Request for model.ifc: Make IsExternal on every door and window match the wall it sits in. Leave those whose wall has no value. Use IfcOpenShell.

First a look at what the model holds.

```python
import ifcopenshell
import ifcopenshell.util.element

model = ifcopenshell.open("model.ifc")
print(model.schema)
seen = {}
for e in model.by_type("IfcDoor") + model.by_type("IfcWindow"):
    if not e.FillsVoids:
        continue
    host = e.FillsVoids[0].RelatingOpeningElement.VoidsElements[0].RelatingBuildingElement
    own = ifcopenshell.util.element.get_pset(e, f"Pset_{e.is_a()[3:].removesuffix('StandardCase')}Common", "IsExternal")
    wall = ifcopenshell.util.element.get_pset(host, "Pset_WallCommon", "IsExternal")
    seen[e.is_a(), own, wall] = seen.get((e.is_a(), own, wall), 0) + 1
for (cls, own, wall), count in sorted(seen.items(), key=str):
    print(count, cls, "IsExternal:", own, "| host wall:", wall)
```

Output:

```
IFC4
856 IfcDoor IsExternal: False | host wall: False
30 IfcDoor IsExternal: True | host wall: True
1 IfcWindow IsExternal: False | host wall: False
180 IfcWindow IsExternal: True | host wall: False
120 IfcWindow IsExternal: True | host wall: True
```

```python
import ifcopenshell
import ifcopenshell.api.pset
import ifcopenshell.util.element

model = ifcopenshell.open("model.ifc")

count = 0
for ifc_class, pset_name in (("IfcDoor", "Pset_DoorCommon"), ("IfcWindow", "Pset_WindowCommon")):
    for e in model.by_type(ifc_class):
        if not e.FillsVoids:
            continue
        host = e.FillsVoids[0].RelatingOpeningElement.VoidsElements[0].RelatingBuildingElement
        external = ifcopenshell.util.element.get_pset(host, "Pset_WallCommon", "IsExternal")
        if external is None or ifcopenshell.util.element.get_pset(e, pset_name, "IsExternal") == external:
            continue
        pset = ifcopenshell.api.pset.add_pset(model, product=e, name=pset_name)
        ifcopenshell.api.pset.edit_pset(model, pset=pset, properties={"IsExternal": external})
        count += 1

print(count, "updated")

model.write("model_edited.ifc")
```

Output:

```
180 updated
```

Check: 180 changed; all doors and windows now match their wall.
